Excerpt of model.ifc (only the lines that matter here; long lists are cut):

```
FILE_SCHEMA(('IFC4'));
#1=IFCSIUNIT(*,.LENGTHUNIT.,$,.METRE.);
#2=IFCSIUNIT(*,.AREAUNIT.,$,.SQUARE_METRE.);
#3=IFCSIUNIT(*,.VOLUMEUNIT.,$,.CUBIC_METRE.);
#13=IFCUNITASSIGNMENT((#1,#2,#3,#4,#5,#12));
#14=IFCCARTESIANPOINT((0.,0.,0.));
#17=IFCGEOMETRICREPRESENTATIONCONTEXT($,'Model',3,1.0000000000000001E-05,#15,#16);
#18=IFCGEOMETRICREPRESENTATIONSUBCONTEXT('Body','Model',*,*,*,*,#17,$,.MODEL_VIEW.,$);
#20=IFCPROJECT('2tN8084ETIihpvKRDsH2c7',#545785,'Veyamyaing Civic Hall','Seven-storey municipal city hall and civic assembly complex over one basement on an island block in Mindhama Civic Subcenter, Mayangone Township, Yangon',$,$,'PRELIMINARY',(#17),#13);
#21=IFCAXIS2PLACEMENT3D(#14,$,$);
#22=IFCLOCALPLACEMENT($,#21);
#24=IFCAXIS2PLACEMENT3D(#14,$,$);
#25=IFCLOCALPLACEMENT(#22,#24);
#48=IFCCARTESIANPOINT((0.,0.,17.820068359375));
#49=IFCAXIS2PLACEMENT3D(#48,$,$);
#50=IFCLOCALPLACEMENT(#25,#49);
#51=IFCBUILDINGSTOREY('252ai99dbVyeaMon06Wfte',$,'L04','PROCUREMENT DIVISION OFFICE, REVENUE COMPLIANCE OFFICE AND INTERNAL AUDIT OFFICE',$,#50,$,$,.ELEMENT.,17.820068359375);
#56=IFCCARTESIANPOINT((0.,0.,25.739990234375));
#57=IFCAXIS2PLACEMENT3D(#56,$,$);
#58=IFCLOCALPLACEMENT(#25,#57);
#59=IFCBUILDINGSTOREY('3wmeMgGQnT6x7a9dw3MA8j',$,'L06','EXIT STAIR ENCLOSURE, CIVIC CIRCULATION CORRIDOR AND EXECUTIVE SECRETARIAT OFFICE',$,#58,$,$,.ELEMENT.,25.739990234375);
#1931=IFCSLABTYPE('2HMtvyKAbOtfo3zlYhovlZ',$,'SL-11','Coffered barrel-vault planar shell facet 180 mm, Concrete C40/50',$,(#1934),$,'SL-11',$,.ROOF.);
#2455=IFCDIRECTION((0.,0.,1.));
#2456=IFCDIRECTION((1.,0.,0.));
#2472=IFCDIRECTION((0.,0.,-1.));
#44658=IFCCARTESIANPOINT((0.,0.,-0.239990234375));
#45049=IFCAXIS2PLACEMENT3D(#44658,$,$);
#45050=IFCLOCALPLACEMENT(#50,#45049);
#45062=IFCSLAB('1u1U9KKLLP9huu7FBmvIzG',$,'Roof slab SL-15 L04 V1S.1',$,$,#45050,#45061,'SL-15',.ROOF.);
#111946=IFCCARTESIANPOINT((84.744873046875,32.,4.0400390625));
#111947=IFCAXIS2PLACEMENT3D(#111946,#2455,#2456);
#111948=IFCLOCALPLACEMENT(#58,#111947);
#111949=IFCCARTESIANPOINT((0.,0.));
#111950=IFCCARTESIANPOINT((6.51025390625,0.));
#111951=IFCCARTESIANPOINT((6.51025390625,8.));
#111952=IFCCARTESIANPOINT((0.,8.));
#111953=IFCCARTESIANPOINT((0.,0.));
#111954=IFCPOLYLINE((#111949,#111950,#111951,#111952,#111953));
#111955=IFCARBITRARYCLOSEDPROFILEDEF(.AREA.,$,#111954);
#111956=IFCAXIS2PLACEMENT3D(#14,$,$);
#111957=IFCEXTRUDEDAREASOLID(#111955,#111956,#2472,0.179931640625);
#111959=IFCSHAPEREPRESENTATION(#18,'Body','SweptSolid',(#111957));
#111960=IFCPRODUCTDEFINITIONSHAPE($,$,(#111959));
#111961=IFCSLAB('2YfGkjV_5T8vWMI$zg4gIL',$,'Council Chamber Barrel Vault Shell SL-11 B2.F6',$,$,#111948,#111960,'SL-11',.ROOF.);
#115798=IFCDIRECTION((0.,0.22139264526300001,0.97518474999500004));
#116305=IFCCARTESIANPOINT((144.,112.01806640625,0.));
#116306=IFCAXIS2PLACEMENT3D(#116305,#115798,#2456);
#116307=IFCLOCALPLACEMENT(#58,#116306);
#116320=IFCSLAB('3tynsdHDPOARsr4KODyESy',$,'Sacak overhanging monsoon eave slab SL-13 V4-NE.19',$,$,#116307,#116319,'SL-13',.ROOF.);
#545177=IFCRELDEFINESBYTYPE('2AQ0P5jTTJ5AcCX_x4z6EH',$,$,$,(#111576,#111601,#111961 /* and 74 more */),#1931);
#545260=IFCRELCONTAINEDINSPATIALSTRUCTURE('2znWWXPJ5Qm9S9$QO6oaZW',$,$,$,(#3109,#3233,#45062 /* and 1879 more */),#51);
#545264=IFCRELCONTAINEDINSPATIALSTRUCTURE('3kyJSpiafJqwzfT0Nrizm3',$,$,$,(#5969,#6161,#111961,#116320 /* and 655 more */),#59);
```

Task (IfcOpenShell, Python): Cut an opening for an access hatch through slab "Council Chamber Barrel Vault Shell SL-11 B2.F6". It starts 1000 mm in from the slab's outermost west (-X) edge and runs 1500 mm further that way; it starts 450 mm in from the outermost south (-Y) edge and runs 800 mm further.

```python
import numpy as np
import ifcopenshell
import ifcopenshell.api.feature
import ifcopenshell.api.geometry
import ifcopenshell.api.root
import ifcopenshell.geom
import ifcopenshell.util.placement
import ifcopenshell.util.representation
import ifcopenshell.util.shape
import ifcopenshell.util.unit

model = ifcopenshell.open("model.ifc")
unit_scale = ifcopenshell.util.unit.calculate_unit_scale(model)
settings = ifcopenshell.geom.settings()


def volume(element):
    """Net volume in cubic metres, openings subtracted."""
    shape = ifcopenshell.geom.create_shape(settings, element)
    return ifcopenshell.util.shape.get_volume(shape.geometry)


slab = model.by_id(111961)
before = volume(slab)

# Extent in the slab's own axes, in metres. The edges named are its -X and -Y sides.
slab_shape = ifcopenshell.geom.create_shape(settings, slab)
vertices = ifcopenshell.util.shape.get_vertices(slab_shape.geometry)
x_min, y_min, bottom = vertices.min(axis=0)
top = vertices[:, 2].max()

opening = ifcopenshell.api.root.create_entity(model, ifc_class="IfcOpeningElement", name="Access hatch opening", predefined_type="OPENING")
context = ifcopenshell.util.representation.get_context(model, "Model", "Body", "MODEL_VIEW")
width, depth = 1.5, 0.8
outline = [(0.0, 0.0), (width, 0.0), (width, depth), (0.0, depth), (0.0, 0.0)]
# Overshoot both faces by 50 mm so the cut is clean.
shape = ifcopenshell.api.geometry.add_slab_representation(
    model, context=context, depth=top - bottom + 0.1, polyline=outline
)
ifcopenshell.api.geometry.assign_representation(model, product=opening, representation=shape)

matrix = ifcopenshell.util.placement.get_local_placement(slab.ObjectPlacement)
matrix[:, 3] = matrix @ np.append(np.array([x_min + 1, y_min + 0.45, bottom - 0.05]) / unit_scale, 1.0)
ifcopenshell.api.geometry.edit_object_placement(model, product=opening, matrix=matrix, is_si=False)
ifcopenshell.api.feature.add_feature(model, feature=opening, element=slab)

after = volume(slab)

print(f"slab volume {before:.3f} -> {after:.3f} m3")

model.write("model_updated.ifc")
```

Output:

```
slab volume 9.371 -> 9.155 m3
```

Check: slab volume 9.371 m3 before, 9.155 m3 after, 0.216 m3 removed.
